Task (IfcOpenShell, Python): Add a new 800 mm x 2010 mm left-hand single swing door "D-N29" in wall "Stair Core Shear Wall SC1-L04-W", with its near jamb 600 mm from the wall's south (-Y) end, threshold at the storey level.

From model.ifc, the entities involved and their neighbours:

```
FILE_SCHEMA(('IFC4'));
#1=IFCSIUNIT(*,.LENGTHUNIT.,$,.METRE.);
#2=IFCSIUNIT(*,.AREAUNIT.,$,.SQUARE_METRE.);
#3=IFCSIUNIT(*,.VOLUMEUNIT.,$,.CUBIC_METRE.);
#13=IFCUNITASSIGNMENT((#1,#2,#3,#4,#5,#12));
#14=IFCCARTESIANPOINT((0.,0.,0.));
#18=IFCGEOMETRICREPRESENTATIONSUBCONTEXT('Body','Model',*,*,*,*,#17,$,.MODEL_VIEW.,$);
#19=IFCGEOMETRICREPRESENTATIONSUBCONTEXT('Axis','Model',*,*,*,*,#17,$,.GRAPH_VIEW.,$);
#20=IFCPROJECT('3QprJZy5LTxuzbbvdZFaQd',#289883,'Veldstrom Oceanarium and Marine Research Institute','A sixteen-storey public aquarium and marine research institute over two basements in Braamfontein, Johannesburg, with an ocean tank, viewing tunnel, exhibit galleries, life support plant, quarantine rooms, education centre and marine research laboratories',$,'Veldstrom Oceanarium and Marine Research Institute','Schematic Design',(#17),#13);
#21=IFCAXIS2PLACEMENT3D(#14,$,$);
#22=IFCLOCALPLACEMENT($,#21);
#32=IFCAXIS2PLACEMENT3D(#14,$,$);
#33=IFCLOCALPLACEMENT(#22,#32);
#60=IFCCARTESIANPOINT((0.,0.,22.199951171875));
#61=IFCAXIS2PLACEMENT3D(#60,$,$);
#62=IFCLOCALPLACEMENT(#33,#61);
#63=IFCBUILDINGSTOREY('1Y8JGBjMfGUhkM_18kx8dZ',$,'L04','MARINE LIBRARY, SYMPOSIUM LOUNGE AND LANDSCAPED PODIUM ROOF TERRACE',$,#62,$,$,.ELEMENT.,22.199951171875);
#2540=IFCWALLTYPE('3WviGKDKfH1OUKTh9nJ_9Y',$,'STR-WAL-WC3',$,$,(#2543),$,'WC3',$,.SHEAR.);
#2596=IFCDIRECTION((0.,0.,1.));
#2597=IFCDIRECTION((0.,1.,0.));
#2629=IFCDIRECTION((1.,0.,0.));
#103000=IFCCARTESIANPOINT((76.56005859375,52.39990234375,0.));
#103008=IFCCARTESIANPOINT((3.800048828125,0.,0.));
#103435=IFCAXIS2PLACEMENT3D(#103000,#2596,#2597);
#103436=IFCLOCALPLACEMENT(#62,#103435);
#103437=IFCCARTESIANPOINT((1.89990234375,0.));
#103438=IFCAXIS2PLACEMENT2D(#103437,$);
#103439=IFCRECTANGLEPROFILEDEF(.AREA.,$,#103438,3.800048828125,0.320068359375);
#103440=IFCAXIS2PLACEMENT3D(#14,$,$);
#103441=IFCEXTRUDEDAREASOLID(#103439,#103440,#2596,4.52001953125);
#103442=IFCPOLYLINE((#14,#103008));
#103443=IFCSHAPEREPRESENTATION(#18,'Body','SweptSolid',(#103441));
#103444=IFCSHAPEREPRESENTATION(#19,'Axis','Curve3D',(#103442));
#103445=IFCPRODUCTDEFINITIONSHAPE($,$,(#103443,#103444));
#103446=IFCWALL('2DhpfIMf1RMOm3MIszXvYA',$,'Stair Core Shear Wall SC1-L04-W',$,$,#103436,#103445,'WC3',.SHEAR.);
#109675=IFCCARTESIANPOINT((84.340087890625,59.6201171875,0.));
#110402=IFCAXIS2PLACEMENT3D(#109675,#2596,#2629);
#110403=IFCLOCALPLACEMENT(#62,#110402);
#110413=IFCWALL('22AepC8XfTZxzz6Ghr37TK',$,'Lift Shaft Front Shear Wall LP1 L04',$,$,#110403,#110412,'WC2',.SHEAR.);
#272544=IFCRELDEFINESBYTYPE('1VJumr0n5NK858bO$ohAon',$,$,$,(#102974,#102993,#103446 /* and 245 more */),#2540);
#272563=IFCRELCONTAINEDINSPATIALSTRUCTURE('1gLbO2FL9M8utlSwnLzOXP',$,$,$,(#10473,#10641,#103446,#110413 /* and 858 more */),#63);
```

```python
import numpy as np
import ifcopenshell
import ifcopenshell.api.feature
import ifcopenshell.api.geometry
import ifcopenshell.api.root
import ifcopenshell.api.spatial
import ifcopenshell.geom
import ifcopenshell.util.element
import ifcopenshell.util.placement
import ifcopenshell.util.representation
import ifcopenshell.util.shape
import ifcopenshell.util.unit

model = ifcopenshell.open("model.ifc")
unit_scale = ifcopenshell.util.unit.calculate_unit_scale(model)
settings = ifcopenshell.geom.settings()


def volume(element):
    """Net volume in cubic metres, openings subtracted."""
    shape = ifcopenshell.geom.create_shape(settings, element)
    return ifcopenshell.util.shape.get_volume(shape.geometry)


wall = model.by_guid("2DhpfIMf1RMOm3MIszXvYA")
storey = ifcopenshell.util.element.get_container(wall, ifc_class="IfcBuildingStorey")
context = ifcopenshell.util.representation.get_context(model, "Model", "Body", "MODEL_VIEW")
before = volume(wall)

width, height, from_end, sill = 0.8, 2.01, 0.6, 0.0  # metres

# The wall runs along its own X axis, and the end named is its -X end.
wall_shape = ifcopenshell.geom.create_shape(settings, wall)
x, y, z = ifcopenshell.util.shape.get_vertices(wall_shape.geometry).T
start = x.min() + from_end
face, thickness = float(y.min()), float(y.max() - y.min())
wall_matrix = ifcopenshell.util.placement.get_local_placement(wall.ObjectPlacement)
level = ifcopenshell.util.placement.get_local_placement(storey.ObjectPlacement)[2, 3]


def in_wall(x, y):
    """Placement at x, y metres in the wall's axes, at sill height."""
    matrix = wall_matrix.copy()
    matrix[:, 3] = wall_matrix @ np.array([x / unit_scale, y / unit_scale, 0.0, 1.0])
    matrix[2, 3] = level + sill / unit_scale
    return matrix


# Opening: a box that overshoots both wall faces by 50 mm.
opening = ifcopenshell.api.root.create_entity(model, ifc_class="IfcOpeningElement", predefined_type="OPENING")
box = ifcopenshell.api.geometry.add_wall_representation(
    model, context=context, length=width, height=height, thickness=thickness + 0.1
)
ifcopenshell.api.geometry.assign_representation(model, product=opening, representation=box)
ifcopenshell.api.geometry.edit_object_placement(model, product=opening, matrix=in_wall(start, face - 0.05), is_si=False)
ifcopenshell.api.feature.add_feature(model, feature=opening, element=wall)

door = ifcopenshell.api.root.create_entity(model, ifc_class="IfcDoor", name="D-N29", predefined_type="DOOR")
door.OverallWidth, door.OverallHeight = width / unit_scale, height / unit_scale
door.OperationType = "SINGLE_SWING_LEFT"
body = ifcopenshell.api.geometry.add_door_representation(
    model,
    context=context,
    overall_width=door.OverallWidth,
    overall_height=door.OverallHeight,
    operation_type="SINGLE_SWING_LEFT",
    lining_properties={"LiningDepth": thickness / unit_scale, "ThresholdDepth": thickness / unit_scale},
)
ifcopenshell.api.geometry.assign_representation(model, product=door, representation=body)
ifcopenshell.api.spatial.assign_container(model, products=[door], relating_structure=storey)
ifcopenshell.api.feature.add_filling(model, opening=opening, element=door)

# The lining spans the wall, so the door starts at the wall face.
ifcopenshell.api.geometry.edit_object_placement(model, product=door, matrix=in_wall(start, face), is_si=False)

after = volume(wall)

print(f"wall volume {before:.3f} -> {after:.3f} m3")

model.write("model_v2.ifc")
```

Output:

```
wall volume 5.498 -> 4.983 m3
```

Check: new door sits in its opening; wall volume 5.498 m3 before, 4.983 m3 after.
